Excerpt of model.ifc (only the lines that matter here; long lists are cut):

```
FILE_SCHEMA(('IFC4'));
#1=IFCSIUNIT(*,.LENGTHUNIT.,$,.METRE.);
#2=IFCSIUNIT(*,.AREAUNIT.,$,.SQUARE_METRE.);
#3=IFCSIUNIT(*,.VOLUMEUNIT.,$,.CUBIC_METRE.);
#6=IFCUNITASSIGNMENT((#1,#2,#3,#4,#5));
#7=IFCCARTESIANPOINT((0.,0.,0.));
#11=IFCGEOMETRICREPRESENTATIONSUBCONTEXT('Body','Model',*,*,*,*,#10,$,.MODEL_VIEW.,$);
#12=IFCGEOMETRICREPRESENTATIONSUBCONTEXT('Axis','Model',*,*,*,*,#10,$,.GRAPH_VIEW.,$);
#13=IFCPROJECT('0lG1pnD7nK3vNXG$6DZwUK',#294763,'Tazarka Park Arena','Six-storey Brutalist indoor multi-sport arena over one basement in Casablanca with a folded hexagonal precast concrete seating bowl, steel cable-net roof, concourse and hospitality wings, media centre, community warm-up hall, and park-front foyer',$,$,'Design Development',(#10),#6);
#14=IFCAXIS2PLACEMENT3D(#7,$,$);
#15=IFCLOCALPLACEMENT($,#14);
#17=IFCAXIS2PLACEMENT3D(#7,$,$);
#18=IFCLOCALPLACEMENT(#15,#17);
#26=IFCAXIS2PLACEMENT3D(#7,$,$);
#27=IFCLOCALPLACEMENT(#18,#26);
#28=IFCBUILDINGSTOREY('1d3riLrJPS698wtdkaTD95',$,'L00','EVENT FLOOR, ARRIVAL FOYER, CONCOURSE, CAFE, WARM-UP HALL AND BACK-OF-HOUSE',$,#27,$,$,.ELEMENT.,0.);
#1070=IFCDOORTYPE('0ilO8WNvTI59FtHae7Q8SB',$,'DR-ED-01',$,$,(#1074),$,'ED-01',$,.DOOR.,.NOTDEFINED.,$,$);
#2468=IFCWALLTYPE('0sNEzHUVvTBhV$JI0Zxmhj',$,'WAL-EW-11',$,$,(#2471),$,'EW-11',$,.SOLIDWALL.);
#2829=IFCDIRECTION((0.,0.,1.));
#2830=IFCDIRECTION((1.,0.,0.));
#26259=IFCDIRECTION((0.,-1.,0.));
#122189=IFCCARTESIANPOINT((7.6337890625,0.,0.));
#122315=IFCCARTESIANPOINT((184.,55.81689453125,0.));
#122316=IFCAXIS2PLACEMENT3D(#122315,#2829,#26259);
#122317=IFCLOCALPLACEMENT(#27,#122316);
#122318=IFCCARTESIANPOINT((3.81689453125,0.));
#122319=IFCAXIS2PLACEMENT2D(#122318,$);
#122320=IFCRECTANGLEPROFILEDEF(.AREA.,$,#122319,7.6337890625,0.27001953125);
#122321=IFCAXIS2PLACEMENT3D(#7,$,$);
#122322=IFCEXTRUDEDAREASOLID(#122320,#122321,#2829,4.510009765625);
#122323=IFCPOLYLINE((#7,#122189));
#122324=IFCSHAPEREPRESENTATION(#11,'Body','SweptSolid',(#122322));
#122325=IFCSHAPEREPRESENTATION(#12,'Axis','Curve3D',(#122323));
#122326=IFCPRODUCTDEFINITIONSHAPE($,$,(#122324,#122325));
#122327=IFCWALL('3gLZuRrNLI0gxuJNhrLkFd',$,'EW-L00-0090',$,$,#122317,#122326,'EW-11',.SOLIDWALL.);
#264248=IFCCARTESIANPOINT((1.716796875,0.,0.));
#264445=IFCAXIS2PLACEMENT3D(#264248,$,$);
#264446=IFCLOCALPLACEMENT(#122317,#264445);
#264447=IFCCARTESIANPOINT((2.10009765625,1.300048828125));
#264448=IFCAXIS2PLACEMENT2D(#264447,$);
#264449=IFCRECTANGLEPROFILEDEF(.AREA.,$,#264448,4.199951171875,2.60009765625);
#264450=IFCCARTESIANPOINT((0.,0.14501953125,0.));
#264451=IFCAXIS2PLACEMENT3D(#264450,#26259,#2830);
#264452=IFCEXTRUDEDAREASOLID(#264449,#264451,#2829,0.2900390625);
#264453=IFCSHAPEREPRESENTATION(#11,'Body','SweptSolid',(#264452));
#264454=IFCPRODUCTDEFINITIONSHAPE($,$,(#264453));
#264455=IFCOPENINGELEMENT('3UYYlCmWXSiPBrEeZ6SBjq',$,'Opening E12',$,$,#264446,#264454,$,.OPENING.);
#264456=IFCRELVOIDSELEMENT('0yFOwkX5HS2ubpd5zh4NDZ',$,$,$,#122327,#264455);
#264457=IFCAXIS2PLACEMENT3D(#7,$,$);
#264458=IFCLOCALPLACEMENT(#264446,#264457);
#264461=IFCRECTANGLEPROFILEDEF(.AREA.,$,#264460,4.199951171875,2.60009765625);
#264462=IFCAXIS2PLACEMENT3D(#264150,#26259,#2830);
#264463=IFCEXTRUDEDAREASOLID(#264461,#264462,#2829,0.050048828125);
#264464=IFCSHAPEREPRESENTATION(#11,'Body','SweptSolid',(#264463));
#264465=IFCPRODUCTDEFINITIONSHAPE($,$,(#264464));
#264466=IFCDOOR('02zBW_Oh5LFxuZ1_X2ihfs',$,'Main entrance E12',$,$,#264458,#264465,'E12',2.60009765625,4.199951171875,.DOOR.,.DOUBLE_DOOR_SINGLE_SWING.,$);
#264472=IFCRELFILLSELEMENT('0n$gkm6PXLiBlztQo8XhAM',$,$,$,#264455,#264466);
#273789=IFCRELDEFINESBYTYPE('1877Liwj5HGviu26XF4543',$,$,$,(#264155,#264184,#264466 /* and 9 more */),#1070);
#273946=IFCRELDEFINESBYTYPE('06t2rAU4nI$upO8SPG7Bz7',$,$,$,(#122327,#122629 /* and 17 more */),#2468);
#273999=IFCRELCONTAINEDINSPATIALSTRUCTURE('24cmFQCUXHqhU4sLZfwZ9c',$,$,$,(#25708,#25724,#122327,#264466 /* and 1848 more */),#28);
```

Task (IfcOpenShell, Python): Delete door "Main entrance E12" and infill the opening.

```python
import ifcopenshell
import ifcopenshell.api.feature
import ifcopenshell.api.root
import ifcopenshell.geom
import ifcopenshell.util.shape

model = ifcopenshell.open("model.ifc")
settings = ifcopenshell.geom.settings()


def volume(element):
    """Net volume in cubic metres, openings subtracted."""
    shape = ifcopenshell.geom.create_shape(settings, element)
    return ifcopenshell.util.shape.get_volume(shape.geometry)


door = model.by_guid("02zBW_Oh5LFxuZ1_X2ihfs")
opening = door.FillsVoids[0].RelatingOpeningElement
wall = opening.VoidsElements[0].RelatingBuildingElement
before = volume(wall)

ifcopenshell.api.root.remove_product(model, product=door)
ifcopenshell.api.feature.remove_feature(model, feature=opening)

after = volume(wall)

print(f"wall volume {before:.3f} -> {after:.3f} m3")

model.write("model-out.ifc")
```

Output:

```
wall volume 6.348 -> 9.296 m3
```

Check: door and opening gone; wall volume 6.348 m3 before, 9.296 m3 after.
